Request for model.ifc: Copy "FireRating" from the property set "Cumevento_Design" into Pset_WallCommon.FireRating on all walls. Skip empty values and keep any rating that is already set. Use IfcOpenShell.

First a look at what the model holds.

```python
import ifcopenshell
import ifcopenshell.util.element

model = ifcopenshell.open("model.ifc")
print(model.schema)
walls = model.by_type("IfcWall")
print(len(walls), "walls")
for e in walls[:8]:
    source = ifcopenshell.util.element.get_pset(e, "Cumevento_Design", "FireRating")
    target = ifcopenshell.util.element.get_pset(e, "Pset_WallCommon", "FireRating")
    print(e.id(), repr(source), repr(target), sep=" | ")
```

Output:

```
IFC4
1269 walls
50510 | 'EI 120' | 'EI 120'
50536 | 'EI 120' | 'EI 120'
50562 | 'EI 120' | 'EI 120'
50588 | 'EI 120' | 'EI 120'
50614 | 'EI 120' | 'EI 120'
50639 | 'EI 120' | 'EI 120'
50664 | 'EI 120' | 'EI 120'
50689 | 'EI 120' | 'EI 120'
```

```python
import ifcopenshell
import ifcopenshell.api.pset
import ifcopenshell.util.element

model = ifcopenshell.open("model.ifc")

count = 0
for e in model.by_type("IfcWall"):
    value = ifcopenshell.util.element.get_pset(e, "Cumevento_Design", "FireRating")
    current = ifcopenshell.util.element.get_pset(e, "Pset_WallCommon", "FireRating")
    if not value or not value.strip() or current:
        continue
    # add_pset returns the element's existing set when there is one.
    pset = ifcopenshell.api.pset.add_pset(model, product=e, name="Pset_WallCommon")
    ifcopenshell.api.pset.edit_pset(model, pset=pset, properties={"FireRating": value})
    count += 1

print(count, "walls updated")

model.write("model_updated.ifc")
```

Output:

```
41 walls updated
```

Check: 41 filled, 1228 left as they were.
